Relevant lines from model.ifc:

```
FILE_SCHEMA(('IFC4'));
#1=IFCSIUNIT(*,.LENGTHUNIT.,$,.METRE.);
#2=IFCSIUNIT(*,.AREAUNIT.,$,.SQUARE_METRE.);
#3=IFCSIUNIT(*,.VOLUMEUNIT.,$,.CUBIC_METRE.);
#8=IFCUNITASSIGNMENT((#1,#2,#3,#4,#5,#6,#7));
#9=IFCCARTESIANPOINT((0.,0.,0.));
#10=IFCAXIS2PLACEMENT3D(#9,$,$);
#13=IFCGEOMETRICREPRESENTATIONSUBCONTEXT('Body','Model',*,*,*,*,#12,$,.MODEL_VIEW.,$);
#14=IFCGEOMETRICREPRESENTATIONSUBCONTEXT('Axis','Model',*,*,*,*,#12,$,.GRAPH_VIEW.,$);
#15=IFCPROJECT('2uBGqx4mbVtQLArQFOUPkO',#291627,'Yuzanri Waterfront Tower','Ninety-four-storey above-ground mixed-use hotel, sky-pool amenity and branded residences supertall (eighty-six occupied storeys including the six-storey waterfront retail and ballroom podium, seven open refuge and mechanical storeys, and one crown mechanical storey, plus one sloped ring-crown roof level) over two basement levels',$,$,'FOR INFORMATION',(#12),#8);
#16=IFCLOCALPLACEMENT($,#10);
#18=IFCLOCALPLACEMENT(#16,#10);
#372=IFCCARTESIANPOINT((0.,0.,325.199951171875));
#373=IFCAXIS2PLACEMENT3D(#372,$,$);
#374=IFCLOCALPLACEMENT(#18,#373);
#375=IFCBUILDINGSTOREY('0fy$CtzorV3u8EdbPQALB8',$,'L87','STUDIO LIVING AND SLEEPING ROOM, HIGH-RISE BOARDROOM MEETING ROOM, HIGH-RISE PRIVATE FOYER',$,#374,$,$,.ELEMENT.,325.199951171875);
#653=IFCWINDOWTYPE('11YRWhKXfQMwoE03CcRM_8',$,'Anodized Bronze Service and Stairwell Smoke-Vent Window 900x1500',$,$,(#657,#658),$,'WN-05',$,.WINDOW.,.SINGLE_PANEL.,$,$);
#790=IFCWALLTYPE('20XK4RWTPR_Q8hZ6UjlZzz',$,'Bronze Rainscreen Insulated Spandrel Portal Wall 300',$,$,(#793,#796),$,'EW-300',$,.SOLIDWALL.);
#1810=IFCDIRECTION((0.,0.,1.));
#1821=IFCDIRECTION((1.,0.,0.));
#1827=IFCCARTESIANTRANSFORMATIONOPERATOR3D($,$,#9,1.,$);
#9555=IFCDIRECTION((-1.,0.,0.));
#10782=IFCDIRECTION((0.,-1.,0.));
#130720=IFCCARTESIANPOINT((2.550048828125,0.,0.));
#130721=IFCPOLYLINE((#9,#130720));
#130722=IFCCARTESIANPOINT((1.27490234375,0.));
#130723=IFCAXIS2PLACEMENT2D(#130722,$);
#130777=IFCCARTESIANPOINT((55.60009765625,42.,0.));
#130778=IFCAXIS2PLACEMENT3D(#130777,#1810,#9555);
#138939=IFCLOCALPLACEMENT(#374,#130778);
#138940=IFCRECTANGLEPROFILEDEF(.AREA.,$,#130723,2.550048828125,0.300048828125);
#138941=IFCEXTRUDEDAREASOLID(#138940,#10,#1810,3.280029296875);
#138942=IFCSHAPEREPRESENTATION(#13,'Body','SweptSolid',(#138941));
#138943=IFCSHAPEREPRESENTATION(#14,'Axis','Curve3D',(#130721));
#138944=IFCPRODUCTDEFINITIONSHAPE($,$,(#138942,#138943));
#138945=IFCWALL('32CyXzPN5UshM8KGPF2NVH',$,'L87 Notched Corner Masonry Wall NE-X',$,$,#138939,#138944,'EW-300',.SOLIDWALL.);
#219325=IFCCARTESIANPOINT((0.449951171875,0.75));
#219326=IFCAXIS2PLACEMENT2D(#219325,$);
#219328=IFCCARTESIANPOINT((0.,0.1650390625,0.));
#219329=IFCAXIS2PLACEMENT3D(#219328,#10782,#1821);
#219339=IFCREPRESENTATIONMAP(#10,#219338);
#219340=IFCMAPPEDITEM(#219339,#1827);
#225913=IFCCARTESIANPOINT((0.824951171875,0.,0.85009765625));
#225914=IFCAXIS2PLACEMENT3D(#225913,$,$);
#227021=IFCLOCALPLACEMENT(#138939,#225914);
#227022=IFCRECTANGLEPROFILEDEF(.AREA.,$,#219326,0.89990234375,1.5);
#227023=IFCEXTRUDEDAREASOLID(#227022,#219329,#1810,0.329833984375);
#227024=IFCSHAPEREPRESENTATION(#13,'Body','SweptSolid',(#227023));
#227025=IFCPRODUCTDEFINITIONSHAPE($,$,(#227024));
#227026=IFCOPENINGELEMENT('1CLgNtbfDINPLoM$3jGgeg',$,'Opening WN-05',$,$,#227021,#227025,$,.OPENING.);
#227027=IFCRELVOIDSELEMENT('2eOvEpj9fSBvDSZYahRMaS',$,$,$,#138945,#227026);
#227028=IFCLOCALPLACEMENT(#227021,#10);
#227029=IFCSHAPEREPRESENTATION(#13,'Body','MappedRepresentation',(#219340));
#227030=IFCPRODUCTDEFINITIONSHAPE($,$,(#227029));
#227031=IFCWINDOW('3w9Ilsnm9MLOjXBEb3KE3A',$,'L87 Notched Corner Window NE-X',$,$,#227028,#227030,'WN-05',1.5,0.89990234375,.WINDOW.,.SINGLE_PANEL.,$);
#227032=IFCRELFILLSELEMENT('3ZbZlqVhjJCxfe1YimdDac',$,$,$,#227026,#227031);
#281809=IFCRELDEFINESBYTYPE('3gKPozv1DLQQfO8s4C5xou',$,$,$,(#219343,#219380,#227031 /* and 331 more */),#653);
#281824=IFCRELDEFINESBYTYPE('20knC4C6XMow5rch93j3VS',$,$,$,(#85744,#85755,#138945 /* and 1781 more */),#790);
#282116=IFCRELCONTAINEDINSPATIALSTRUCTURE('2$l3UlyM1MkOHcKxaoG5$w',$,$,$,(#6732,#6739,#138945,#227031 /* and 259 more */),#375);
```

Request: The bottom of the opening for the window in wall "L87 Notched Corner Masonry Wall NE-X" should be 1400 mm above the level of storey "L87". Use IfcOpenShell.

```python
import numpy as np
import ifcopenshell
import ifcopenshell.api.geometry
import ifcopenshell.geom
import ifcopenshell.util.element
import ifcopenshell.util.placement
import ifcopenshell.util.shape
import ifcopenshell.util.unit

model = ifcopenshell.open("model.ifc")
unit_scale = ifcopenshell.util.unit.calculate_unit_scale(model)

window = model.by_guid("3w9Ilsnm9MLOjXBEb3KE3A")
opening = window.FillsVoids[0].RelatingOpeningElement
storey = ifcopenshell.util.element.get_container(window, ifc_class="IfcBuildingStorey")
level = ifcopenshell.util.placement.get_local_placement(storey.ObjectPlacement)[2, 3]

# The opening's origin need not be at the sill, so measure its lowest point.
shape = ifcopenshell.geom.create_shape(ifcopenshell.geom.settings(), opening)
bottom = ifcopenshell.util.shape.get_shape_bottom_elevation(shape, shape.geometry) / unit_scale
dz = level + 1.4 - bottom

shift = np.array([0.0, 0.0, dz])
# The window is placed relative to its opening, so it follows when the opening moves.
matrix = ifcopenshell.util.placement.get_local_placement(opening.ObjectPlacement)
matrix[:3, 3] += shift
ifcopenshell.api.geometry.edit_object_placement(
    model, product=opening, matrix=matrix, is_si=False, should_transform_children=True
)

print(f"moved by {dz * unit_scale:+.3f} m")

model.write("model_edited.ifc")
```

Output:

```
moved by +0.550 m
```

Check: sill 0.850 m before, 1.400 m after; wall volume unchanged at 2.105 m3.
